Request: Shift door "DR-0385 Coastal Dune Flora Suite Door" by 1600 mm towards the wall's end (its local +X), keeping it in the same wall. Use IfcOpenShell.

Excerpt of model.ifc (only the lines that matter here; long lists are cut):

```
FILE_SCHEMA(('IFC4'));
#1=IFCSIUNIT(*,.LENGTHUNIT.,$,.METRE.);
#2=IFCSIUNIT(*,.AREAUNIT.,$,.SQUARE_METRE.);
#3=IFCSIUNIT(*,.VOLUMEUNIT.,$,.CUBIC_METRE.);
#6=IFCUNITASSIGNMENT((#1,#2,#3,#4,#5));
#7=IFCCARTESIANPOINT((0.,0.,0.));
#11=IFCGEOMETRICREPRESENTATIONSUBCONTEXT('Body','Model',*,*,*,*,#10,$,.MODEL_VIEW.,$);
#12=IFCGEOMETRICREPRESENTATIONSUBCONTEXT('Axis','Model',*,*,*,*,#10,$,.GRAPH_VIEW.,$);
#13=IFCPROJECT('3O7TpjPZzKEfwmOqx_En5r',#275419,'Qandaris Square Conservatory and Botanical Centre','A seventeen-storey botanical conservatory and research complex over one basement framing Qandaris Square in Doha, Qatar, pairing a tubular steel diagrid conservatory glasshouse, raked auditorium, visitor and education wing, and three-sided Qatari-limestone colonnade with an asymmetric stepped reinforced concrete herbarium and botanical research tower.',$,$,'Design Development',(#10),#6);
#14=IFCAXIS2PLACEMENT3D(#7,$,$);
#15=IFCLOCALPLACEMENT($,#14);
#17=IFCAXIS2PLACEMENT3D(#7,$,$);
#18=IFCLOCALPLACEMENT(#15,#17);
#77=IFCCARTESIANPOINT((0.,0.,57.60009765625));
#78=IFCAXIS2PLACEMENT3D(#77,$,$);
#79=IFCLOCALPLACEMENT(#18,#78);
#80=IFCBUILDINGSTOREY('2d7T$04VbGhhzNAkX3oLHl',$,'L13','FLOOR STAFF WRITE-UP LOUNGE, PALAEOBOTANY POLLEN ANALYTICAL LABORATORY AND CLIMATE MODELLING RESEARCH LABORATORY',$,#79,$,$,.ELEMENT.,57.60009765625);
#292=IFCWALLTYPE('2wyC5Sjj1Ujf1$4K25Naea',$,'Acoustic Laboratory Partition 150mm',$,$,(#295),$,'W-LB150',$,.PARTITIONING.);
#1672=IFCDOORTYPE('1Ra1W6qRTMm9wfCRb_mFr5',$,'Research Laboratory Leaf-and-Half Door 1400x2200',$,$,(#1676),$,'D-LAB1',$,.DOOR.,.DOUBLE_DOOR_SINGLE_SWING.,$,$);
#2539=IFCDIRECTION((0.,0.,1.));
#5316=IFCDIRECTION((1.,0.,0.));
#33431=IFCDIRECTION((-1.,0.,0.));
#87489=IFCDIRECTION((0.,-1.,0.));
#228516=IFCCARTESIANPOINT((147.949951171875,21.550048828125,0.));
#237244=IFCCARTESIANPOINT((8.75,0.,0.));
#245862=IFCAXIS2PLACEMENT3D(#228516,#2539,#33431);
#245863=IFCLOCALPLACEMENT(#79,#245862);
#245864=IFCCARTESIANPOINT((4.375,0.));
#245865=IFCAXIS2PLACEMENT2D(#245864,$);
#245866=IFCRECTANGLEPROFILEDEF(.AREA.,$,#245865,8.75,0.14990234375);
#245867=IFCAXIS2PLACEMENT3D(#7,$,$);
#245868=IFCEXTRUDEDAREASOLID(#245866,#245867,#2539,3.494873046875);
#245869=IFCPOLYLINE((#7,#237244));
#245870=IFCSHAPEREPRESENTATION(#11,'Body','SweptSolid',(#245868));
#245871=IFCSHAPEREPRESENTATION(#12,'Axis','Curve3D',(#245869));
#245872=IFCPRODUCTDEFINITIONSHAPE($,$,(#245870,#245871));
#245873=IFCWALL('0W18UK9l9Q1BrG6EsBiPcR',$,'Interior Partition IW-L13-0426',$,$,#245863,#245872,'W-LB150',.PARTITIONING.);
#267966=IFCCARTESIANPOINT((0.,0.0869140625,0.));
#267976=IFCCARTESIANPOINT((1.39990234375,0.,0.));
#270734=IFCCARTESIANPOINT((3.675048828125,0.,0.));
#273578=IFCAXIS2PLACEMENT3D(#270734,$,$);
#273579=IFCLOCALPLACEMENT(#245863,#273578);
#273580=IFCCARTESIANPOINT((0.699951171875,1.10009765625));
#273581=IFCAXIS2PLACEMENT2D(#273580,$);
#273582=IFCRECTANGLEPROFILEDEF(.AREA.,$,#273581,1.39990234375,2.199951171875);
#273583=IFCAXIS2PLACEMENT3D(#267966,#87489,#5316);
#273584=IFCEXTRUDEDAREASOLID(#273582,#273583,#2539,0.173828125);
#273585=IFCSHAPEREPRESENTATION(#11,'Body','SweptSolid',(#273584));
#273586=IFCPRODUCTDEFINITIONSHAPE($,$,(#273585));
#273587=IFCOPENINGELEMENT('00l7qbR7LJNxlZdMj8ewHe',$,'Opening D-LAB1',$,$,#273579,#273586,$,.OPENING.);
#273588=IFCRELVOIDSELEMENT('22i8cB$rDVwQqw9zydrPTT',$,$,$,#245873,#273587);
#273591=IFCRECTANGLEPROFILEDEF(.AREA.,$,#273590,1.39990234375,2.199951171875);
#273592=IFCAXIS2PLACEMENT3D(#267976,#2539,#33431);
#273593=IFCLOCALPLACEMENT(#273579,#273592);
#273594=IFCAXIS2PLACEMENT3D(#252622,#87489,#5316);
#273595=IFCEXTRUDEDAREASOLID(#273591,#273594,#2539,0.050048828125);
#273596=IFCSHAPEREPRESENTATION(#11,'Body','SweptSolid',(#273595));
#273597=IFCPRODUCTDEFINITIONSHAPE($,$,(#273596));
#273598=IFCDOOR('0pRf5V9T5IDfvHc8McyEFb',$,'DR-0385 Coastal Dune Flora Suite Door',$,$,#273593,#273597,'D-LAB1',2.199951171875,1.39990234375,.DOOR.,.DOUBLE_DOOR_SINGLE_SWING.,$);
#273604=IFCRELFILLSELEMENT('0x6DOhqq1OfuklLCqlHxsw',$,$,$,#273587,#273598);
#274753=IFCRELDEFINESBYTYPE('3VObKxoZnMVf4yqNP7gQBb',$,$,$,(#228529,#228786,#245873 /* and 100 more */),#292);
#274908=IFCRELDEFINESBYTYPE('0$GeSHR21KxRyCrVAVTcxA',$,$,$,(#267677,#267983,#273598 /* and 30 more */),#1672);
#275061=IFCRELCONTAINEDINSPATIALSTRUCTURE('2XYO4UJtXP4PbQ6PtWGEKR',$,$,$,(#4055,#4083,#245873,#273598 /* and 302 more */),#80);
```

```python
import ifcopenshell
import ifcopenshell.api.geometry
import ifcopenshell.util.placement

model = ifcopenshell.open("model.ifc")

door = model.by_guid("0pRf5V9T5IDfvHc8McyEFb")
opening = door.FillsVoids[0].RelatingOpeningElement
wall = opening.VoidsElements[0].RelatingBuildingElement

wall_matrix = ifcopenshell.util.placement.get_local_placement(wall.ObjectPlacement)
shift = wall_matrix[:3, 0] * 1.6
before = ifcopenshell.util.placement.get_local_placement(door.ObjectPlacement)[:3, 3].copy()

# The door is placed relative to its opening, so it follows when the opening moves.
matrix = ifcopenshell.util.placement.get_local_placement(opening.ObjectPlacement)
matrix[:3, 3] += shift
ifcopenshell.api.geometry.edit_object_placement(
    model, product=opening, matrix=matrix, is_si=False, should_transform_children=True
)

after = ifcopenshell.util.placement.get_local_placement(door.ObjectPlacement)[:3, 3]
print("door moved by", (after - before).round(3) + 0.0)

model.write("model_updated.ifc")
```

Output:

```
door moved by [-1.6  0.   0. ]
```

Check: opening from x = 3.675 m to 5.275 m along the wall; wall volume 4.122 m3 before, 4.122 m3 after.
